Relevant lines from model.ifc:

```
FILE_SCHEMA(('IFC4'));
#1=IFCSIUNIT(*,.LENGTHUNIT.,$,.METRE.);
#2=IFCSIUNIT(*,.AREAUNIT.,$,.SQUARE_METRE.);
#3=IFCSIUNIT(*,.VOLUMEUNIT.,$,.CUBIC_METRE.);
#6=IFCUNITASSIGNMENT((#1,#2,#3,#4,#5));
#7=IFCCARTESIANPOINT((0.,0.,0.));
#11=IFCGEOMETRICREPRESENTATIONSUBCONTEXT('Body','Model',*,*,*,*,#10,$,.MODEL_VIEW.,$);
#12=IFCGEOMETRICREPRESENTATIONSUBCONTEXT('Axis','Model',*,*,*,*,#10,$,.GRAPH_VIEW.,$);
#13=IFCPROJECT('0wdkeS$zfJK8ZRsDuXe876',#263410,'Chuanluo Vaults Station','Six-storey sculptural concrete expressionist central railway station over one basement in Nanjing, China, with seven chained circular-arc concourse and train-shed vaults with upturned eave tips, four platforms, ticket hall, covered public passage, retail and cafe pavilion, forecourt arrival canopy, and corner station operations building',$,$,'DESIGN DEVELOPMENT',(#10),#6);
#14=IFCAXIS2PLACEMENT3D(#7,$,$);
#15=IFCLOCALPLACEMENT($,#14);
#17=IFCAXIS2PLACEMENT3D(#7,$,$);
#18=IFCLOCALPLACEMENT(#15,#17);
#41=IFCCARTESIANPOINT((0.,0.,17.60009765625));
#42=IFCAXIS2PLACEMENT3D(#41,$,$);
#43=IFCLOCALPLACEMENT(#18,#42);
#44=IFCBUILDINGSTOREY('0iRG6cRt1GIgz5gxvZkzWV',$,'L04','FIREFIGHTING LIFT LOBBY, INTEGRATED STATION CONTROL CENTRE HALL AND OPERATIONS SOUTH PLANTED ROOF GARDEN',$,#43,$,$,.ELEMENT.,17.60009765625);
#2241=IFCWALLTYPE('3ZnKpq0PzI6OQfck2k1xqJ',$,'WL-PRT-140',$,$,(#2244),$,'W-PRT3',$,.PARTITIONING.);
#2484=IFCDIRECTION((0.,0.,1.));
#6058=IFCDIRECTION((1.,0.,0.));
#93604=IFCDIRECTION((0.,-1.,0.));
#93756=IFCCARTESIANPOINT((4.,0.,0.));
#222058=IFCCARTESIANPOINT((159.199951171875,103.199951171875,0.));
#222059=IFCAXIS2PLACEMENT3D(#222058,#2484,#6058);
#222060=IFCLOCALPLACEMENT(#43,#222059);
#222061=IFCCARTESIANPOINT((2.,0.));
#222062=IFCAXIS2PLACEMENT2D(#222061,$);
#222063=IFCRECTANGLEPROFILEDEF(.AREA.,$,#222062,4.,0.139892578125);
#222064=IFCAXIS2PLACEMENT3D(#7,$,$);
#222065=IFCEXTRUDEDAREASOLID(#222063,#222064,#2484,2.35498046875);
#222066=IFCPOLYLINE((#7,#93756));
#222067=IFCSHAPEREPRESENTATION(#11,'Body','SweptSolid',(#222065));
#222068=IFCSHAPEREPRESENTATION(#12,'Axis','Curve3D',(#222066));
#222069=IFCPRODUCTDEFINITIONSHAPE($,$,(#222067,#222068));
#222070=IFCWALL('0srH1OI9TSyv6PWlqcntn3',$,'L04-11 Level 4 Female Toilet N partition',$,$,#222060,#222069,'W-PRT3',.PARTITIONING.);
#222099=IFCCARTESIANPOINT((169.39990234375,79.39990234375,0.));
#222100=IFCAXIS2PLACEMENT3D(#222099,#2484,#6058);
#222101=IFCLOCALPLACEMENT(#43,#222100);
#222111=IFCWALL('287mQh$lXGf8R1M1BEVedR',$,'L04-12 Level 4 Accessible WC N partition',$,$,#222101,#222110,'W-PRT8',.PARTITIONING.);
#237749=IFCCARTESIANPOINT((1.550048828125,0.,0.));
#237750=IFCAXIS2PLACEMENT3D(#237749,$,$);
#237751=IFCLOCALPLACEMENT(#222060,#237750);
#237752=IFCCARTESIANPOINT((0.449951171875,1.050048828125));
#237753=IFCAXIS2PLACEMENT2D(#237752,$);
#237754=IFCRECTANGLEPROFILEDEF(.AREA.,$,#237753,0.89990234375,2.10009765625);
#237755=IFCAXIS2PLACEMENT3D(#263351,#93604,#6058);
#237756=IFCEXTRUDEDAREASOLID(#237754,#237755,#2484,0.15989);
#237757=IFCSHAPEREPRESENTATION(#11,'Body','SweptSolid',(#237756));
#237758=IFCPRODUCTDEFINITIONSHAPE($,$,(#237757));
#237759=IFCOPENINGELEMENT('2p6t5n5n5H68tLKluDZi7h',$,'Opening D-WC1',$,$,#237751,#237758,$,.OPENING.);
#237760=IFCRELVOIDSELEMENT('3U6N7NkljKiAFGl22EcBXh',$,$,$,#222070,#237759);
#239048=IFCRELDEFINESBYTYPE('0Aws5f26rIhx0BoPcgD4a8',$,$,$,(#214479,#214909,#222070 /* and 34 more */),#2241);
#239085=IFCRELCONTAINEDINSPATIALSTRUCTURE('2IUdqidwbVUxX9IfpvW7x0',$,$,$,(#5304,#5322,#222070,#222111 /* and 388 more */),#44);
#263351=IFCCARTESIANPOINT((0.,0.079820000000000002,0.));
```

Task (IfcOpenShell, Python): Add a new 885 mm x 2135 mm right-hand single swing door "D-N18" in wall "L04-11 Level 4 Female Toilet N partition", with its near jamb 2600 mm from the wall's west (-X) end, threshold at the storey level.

```python
import numpy as np
import ifcopenshell
import ifcopenshell.api.feature
import ifcopenshell.api.geometry
import ifcopenshell.api.root
import ifcopenshell.api.spatial
import ifcopenshell.geom
import ifcopenshell.util.element
import ifcopenshell.util.placement
import ifcopenshell.util.representation
import ifcopenshell.util.shape
import ifcopenshell.util.unit

model = ifcopenshell.open("model.ifc")
unit_scale = ifcopenshell.util.unit.calculate_unit_scale(model)
settings = ifcopenshell.geom.settings()


def volume(element):
    """Net volume in cubic metres, openings subtracted."""
    shape = ifcopenshell.geom.create_shape(settings, element)
    return ifcopenshell.util.shape.get_volume(shape.geometry)


wall = model.by_guid("0srH1OI9TSyv6PWlqcntn3")
storey = ifcopenshell.util.element.get_container(wall, ifc_class="IfcBuildingStorey")
context = ifcopenshell.util.representation.get_context(model, "Model", "Body", "MODEL_VIEW")
before = volume(wall)

width, height, from_end, sill = 0.885, 2.135, 2.6, 0.0  # metres

# The wall runs along its own X axis, and the end named is its -X end.
wall_shape = ifcopenshell.geom.create_shape(settings, wall)
x, y, z = ifcopenshell.util.shape.get_vertices(wall_shape.geometry).T
start = x.min() + from_end
face, thickness = float(y.min()), float(y.max() - y.min())
wall_matrix = ifcopenshell.util.placement.get_local_placement(wall.ObjectPlacement)
level = ifcopenshell.util.placement.get_local_placement(storey.ObjectPlacement)[2, 3]


def in_wall(x, y):
    """Placement at x, y metres in the wall's axes, at sill height."""
    matrix = wall_matrix.copy()
    matrix[:, 3] = wall_matrix @ np.array([x / unit_scale, y / unit_scale, 0.0, 1.0])
    matrix[2, 3] = level + sill / unit_scale
    return matrix


# Opening: a box that overshoots both wall faces by 50 mm.
opening = ifcopenshell.api.root.create_entity(model, ifc_class="IfcOpeningElement", predefined_type="OPENING")
box = ifcopenshell.api.geometry.add_wall_representation(
    model, context=context, length=width, height=height, thickness=thickness + 0.1
)
ifcopenshell.api.geometry.assign_representation(model, product=opening, representation=box)
ifcopenshell.api.geometry.edit_object_placement(model, product=opening, matrix=in_wall(start, face - 0.05), is_si=False)
ifcopenshell.api.feature.add_feature(model, feature=opening, element=wall)

door = ifcopenshell.api.root.create_entity(model, ifc_class="IfcDoor", name="D-N18", predefined_type="DOOR")
door.OverallWidth, door.OverallHeight = width / unit_scale, height / unit_scale
door.OperationType = "SINGLE_SWING_RIGHT"
body = ifcopenshell.api.geometry.add_door_representation(
    model,
    context=context,
    overall_width=door.OverallWidth,
    overall_height=door.OverallHeight,
    operation_type="SINGLE_SWING_RIGHT",
    lining_properties={"LiningDepth": thickness / unit_scale, "ThresholdDepth": thickness / unit_scale},
)
ifcopenshell.api.geometry.assign_representation(model, product=door, representation=body)
ifcopenshell.api.spatial.assign_container(model, products=[door], relating_structure=storey)
ifcopenshell.api.feature.add_filling(model, opening=opening, element=door)

# The lining spans the wall, so the door starts at the wall face.
ifcopenshell.api.geometry.edit_object_placement(model, product=door, matrix=in_wall(start, face), is_si=False)

after = volume(wall)

print(f"wall volume {before:.3f} -> {after:.3f} m3")

model.write("model_updated.ifc")
```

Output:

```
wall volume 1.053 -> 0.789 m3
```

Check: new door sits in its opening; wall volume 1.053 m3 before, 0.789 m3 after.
